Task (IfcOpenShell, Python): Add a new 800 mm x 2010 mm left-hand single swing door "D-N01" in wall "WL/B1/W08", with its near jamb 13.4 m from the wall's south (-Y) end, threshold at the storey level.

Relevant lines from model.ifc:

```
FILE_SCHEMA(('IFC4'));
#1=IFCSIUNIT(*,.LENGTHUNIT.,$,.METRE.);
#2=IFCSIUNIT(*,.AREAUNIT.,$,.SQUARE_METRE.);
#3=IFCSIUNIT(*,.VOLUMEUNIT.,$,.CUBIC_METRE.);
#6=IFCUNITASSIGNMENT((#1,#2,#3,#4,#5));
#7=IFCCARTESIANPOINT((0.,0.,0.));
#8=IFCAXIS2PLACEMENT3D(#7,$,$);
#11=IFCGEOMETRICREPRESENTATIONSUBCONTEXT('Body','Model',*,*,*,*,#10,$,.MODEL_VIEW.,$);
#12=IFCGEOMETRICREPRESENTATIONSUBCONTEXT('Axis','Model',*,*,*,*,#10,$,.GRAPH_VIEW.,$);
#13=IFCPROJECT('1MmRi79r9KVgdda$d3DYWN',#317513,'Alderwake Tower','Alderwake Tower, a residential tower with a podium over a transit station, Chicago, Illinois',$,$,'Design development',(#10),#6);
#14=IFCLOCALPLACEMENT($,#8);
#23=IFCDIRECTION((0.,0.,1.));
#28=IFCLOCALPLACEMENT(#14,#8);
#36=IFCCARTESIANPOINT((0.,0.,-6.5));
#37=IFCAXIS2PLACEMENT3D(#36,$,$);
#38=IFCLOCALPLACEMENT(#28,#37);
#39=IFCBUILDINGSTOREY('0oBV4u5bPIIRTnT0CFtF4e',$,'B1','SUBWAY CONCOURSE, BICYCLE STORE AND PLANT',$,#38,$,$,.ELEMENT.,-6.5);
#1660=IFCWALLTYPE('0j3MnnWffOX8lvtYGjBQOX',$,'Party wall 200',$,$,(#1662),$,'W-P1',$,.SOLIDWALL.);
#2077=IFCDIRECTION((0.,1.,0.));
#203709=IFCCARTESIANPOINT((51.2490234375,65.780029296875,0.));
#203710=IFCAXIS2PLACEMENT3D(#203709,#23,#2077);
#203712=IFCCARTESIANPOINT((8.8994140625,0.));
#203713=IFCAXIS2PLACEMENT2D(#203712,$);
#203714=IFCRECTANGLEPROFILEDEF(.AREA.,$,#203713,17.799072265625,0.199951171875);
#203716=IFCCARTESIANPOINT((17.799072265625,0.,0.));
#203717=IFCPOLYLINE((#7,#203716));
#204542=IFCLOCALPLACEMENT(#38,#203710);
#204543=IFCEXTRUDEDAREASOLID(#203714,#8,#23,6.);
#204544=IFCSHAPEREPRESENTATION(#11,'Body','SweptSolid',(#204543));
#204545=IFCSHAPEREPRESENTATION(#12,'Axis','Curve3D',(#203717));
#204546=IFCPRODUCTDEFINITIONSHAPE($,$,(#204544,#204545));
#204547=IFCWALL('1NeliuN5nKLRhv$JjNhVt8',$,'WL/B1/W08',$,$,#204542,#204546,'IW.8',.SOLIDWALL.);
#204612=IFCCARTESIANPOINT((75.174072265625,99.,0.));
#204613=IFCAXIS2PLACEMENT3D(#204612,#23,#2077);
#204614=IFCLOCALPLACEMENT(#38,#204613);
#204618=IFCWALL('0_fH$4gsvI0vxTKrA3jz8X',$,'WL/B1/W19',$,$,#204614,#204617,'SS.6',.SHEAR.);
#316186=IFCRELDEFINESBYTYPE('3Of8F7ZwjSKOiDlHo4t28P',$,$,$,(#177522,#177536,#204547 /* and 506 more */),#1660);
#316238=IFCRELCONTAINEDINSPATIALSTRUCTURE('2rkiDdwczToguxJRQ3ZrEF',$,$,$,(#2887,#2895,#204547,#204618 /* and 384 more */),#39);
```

```python
import numpy as np
import ifcopenshell
import ifcopenshell.api.feature
import ifcopenshell.api.geometry
import ifcopenshell.api.root
import ifcopenshell.api.spatial
import ifcopenshell.geom
import ifcopenshell.util.element
import ifcopenshell.util.placement
import ifcopenshell.util.representation
import ifcopenshell.util.shape
import ifcopenshell.util.unit

model = ifcopenshell.open("model.ifc")
unit_scale = ifcopenshell.util.unit.calculate_unit_scale(model)
settings = ifcopenshell.geom.settings()


def volume(element):
    """Net volume in cubic metres, openings subtracted."""
    shape = ifcopenshell.geom.create_shape(settings, element)
    return ifcopenshell.util.shape.get_volume(shape.geometry)


wall = model.by_guid("1NeliuN5nKLRhv$JjNhVt8")
storey = ifcopenshell.util.element.get_container(wall, ifc_class="IfcBuildingStorey")
context = ifcopenshell.util.representation.get_context(model, "Model", "Body", "MODEL_VIEW")
before = volume(wall)

width, height, from_end, sill = 0.8, 2.01, 13.4, 0.0  # metres

# The wall runs along its own X axis, and the end named is its -X end.
wall_shape = ifcopenshell.geom.create_shape(settings, wall)
x, y, z = ifcopenshell.util.shape.get_vertices(wall_shape.geometry).T
start = x.min() + from_end
face, thickness = float(y.min()), float(y.max() - y.min())
wall_matrix = ifcopenshell.util.placement.get_local_placement(wall.ObjectPlacement)
level = ifcopenshell.util.placement.get_local_placement(storey.ObjectPlacement)[2, 3]


def in_wall(x, y):
    """Placement at x, y metres in the wall's axes, at sill height."""
    matrix = wall_matrix.copy()
    matrix[:, 3] = wall_matrix @ np.array([x / unit_scale, y / unit_scale, 0.0, 1.0])
    matrix[2, 3] = level + sill / unit_scale
    return matrix


# Opening: a box that overshoots both wall faces by 50 mm.
opening = ifcopenshell.api.root.create_entity(model, ifc_class="IfcOpeningElement", predefined_type="OPENING")
box = ifcopenshell.api.geometry.add_wall_representation(
    model, context=context, length=width, height=height, thickness=thickness + 0.1
)
ifcopenshell.api.geometry.assign_representation(model, product=opening, representation=box)
ifcopenshell.api.geometry.edit_object_placement(model, product=opening, matrix=in_wall(start, face - 0.05), is_si=False)
ifcopenshell.api.feature.add_feature(model, feature=opening, element=wall)

door = ifcopenshell.api.root.create_entity(model, ifc_class="IfcDoor", name="D-N01", predefined_type="DOOR")
door.OverallWidth, door.OverallHeight = width / unit_scale, height / unit_scale
door.OperationType = "SINGLE_SWING_LEFT"
body = ifcopenshell.api.geometry.add_door_representation(
    model,
    context=context,
    overall_width=door.OverallWidth,
    overall_height=door.OverallHeight,
    operation_type="SINGLE_SWING_LEFT",
    lining_properties={"LiningDepth": thickness / unit_scale, "ThresholdDepth": thickness / unit_scale},
)
ifcopenshell.api.geometry.assign_representation(model, product=door, representation=body)
ifcopenshell.api.spatial.assign_container(model, products=[door], relating_structure=storey)
ifcopenshell.api.feature.add_filling(model, opening=opening, element=door)

# The lining spans the wall, so the door starts at the wall face.
ifcopenshell.api.geometry.edit_object_placement(model, product=door, matrix=in_wall(start, face), is_si=False)

after = volume(wall)

print(f"wall volume {before:.3f} -> {after:.3f} m3")

model.write("model_updated.ifc")
```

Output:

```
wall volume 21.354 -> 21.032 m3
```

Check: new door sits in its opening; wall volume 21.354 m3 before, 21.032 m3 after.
